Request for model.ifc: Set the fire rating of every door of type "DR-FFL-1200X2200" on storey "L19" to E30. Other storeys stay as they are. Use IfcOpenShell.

First a look at what the model holds.

```python
import ifcopenshell
import ifcopenshell.util.element

model = ifcopenshell.open("model.ifc")
print(model.schema)
storey = next(s for s in model.by_type("IfcBuildingStorey") if s.Name == "L19")
doors = [e for e in ifcopenshell.util.element.get_decomposition(storey) if e.is_a("IfcDoor")]
seen = {}
for e in doors:
    element_type = ifcopenshell.util.element.get_type(e)
    key = (element_type.Name if element_type != e and element_type else None, ifcopenshell.util.element.get_pset(e, "Pset_DoorCommon", "FireRating"))
    seen[key] = seen.get(key, 0) + 1
for (name, value), count in sorted(seen.items(), key=str):
    print(count, "x", name, "|", value)
```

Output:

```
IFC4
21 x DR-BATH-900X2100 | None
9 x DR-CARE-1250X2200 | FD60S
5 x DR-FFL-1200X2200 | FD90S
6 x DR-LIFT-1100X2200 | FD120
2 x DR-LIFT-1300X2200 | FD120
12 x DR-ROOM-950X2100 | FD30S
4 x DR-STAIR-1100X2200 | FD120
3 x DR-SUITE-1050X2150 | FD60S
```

```python
import ifcopenshell
import ifcopenshell.api.pset
import ifcopenshell.util.element

model = ifcopenshell.open("model.ifc")

storey = next(s for s in model.by_type("IfcBuildingStorey") if s.Name == "L19")
doors = [e for e in ifcopenshell.util.element.get_decomposition(storey) if e.is_a("IfcDoor")]

count = 0
for e in doors:
    element_type = ifcopenshell.util.element.get_type(e)
    if element_type in (None, e) or element_type.Name != "DR-FFL-1200X2200":
        continue
    found = ifcopenshell.util.element.get_pset(e, "Pset_DoorCommon", should_inherit=False)
    if found:
        pset = model.by_id(found["id"])
        if len(ifcopenshell.util.element.get_elements_by_pset(pset)) > 1:
            pset = ifcopenshell.api.pset.unshare_pset(model, products=[e], pset=pset)[0]
    else:
        pset = ifcopenshell.api.pset.add_pset(model, product=e, name="Pset_DoorCommon")
    ifcopenshell.api.pset.edit_pset(model, pset=pset, properties={"FireRating": "E30"})
    count += 1

print(count, "doors updated")

model.write("model_updated.ifc")
```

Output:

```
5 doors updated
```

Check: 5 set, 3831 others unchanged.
